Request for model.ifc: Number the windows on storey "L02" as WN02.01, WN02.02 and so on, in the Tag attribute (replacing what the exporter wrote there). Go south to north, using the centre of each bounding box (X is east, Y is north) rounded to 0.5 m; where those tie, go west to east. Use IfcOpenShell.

First a look at what the model holds.

```python
import ifcopenshell
import ifcopenshell.util.element
import ifcopenshell.util.placement

model = ifcopenshell.open("model.ifc")
print(model.schema)
storey = next(s for s in model.by_type("IfcBuildingStorey") if s.Name == "L02")
windows = [e for e in ifcopenshell.util.element.get_decomposition(storey) if e.is_a("IfcWindow")]
for e in sorted(windows, key=lambda e: e.id()):
    origin = ifcopenshell.util.placement.get_local_placement(e.ObjectPlacement)[:3, 3]
    print(e.id(), e.Tag, e.Name, origin.round(2) + 0.0, sep=" | ")
```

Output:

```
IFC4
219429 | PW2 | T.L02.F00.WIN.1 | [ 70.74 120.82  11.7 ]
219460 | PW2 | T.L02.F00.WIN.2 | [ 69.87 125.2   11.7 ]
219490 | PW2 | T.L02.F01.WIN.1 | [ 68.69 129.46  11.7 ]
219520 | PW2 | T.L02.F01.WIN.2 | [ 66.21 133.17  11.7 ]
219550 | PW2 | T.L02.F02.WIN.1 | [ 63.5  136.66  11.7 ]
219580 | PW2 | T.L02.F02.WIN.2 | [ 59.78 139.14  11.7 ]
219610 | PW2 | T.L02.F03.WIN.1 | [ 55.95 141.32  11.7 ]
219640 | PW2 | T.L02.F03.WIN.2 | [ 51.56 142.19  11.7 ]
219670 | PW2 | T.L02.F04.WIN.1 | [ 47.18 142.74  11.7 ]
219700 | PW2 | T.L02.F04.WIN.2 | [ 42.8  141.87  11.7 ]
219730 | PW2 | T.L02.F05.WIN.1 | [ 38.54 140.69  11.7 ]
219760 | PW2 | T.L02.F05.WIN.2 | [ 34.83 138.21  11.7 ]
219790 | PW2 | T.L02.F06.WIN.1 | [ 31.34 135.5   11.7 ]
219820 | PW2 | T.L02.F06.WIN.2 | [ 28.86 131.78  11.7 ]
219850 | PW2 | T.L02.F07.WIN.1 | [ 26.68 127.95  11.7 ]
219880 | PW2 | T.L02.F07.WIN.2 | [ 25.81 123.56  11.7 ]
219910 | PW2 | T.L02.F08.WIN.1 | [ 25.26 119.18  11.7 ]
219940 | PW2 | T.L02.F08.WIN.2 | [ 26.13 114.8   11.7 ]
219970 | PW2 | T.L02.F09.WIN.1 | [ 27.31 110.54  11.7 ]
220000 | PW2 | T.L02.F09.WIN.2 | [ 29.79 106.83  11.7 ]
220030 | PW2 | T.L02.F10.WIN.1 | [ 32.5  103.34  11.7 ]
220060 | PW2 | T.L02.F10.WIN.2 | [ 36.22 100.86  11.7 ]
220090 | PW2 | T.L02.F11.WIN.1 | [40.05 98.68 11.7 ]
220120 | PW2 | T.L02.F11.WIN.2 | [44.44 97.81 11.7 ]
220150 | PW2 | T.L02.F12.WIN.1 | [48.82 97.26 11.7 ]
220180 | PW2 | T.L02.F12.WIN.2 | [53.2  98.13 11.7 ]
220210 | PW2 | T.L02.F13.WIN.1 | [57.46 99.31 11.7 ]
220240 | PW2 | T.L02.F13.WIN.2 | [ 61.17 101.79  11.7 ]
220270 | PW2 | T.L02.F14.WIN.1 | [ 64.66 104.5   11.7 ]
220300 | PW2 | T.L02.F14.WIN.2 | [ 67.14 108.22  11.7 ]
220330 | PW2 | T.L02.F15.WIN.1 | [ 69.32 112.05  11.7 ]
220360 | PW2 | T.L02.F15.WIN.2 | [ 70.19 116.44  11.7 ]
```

```python
import ifcopenshell
import ifcopenshell.geom
import ifcopenshell.util.element
import ifcopenshell.util.shape

model = ifcopenshell.open("model.ifc")
settings = ifcopenshell.geom.settings()
settings.set("use-world-coords", True)


def centre(element):
    shape = ifcopenshell.geom.create_shape(settings, element)
    return ifcopenshell.util.shape.get_bbox_centroid(shape.geometry)


storey = next(s for s in model.by_type("IfcBuildingStorey") if s.Name == "L02")
windows = [e for e in ifcopenshell.util.element.get_decomposition(storey) if e.is_a("IfcWindow")]

# Insertion points can sit at a corner or the storey origin, so sort by the geometry (in metres).
centres = {e: centre(e) for e in windows}
windows.sort(key=lambda e: (round(centres[e][1] / 0.5), centres[e][0]))

for i, e in enumerate(windows, start=1):
    number = f"WN02.{i:02d}"
    e.Tag = number
    print(e.id(), number)

model.write("model_edited.ifc")
```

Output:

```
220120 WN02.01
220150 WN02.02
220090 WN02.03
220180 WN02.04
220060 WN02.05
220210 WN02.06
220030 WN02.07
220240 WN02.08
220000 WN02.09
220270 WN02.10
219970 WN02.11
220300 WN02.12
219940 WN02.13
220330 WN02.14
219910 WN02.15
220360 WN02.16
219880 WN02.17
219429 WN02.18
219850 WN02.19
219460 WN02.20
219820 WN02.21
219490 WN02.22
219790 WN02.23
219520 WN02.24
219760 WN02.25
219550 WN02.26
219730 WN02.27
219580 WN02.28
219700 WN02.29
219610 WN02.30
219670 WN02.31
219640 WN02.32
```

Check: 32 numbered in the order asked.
